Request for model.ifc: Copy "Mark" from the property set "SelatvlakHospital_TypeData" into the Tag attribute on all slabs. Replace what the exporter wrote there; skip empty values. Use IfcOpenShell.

First a look at what the model holds.

```python
import ifcopenshell
import ifcopenshell.util.element

model = ifcopenshell.open("model.ifc")
print(model.schema)
slabs = model.by_type("IfcSlab")
print(len(slabs), "slabs")
for e in slabs[:8]:
    source = ifcopenshell.util.element.get_pset(e, "SelatvlakHospital_TypeData", "Mark")
    target = e.Tag
    print(e.id(), repr(source), repr(target), sep=" | ")
```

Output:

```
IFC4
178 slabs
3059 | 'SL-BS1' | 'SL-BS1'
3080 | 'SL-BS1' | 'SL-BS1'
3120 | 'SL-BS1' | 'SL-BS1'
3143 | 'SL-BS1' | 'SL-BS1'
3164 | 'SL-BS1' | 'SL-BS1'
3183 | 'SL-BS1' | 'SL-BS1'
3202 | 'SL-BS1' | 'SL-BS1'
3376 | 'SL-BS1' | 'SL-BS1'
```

```python
import ifcopenshell
import ifcopenshell.util.element

model = ifcopenshell.open("model.ifc")

count = 0
for e in model.by_type("IfcSlab"):
    value = ifcopenshell.util.element.get_pset(e, "SelatvlakHospital_TypeData", "Mark")
    current = e.Tag
    if not value or not value.strip() or current == value:
        continue
    e.Tag = value
    count += 1

print(count, "slabs updated")

model.write("model_edited.ifc")
```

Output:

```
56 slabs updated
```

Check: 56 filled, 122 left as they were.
